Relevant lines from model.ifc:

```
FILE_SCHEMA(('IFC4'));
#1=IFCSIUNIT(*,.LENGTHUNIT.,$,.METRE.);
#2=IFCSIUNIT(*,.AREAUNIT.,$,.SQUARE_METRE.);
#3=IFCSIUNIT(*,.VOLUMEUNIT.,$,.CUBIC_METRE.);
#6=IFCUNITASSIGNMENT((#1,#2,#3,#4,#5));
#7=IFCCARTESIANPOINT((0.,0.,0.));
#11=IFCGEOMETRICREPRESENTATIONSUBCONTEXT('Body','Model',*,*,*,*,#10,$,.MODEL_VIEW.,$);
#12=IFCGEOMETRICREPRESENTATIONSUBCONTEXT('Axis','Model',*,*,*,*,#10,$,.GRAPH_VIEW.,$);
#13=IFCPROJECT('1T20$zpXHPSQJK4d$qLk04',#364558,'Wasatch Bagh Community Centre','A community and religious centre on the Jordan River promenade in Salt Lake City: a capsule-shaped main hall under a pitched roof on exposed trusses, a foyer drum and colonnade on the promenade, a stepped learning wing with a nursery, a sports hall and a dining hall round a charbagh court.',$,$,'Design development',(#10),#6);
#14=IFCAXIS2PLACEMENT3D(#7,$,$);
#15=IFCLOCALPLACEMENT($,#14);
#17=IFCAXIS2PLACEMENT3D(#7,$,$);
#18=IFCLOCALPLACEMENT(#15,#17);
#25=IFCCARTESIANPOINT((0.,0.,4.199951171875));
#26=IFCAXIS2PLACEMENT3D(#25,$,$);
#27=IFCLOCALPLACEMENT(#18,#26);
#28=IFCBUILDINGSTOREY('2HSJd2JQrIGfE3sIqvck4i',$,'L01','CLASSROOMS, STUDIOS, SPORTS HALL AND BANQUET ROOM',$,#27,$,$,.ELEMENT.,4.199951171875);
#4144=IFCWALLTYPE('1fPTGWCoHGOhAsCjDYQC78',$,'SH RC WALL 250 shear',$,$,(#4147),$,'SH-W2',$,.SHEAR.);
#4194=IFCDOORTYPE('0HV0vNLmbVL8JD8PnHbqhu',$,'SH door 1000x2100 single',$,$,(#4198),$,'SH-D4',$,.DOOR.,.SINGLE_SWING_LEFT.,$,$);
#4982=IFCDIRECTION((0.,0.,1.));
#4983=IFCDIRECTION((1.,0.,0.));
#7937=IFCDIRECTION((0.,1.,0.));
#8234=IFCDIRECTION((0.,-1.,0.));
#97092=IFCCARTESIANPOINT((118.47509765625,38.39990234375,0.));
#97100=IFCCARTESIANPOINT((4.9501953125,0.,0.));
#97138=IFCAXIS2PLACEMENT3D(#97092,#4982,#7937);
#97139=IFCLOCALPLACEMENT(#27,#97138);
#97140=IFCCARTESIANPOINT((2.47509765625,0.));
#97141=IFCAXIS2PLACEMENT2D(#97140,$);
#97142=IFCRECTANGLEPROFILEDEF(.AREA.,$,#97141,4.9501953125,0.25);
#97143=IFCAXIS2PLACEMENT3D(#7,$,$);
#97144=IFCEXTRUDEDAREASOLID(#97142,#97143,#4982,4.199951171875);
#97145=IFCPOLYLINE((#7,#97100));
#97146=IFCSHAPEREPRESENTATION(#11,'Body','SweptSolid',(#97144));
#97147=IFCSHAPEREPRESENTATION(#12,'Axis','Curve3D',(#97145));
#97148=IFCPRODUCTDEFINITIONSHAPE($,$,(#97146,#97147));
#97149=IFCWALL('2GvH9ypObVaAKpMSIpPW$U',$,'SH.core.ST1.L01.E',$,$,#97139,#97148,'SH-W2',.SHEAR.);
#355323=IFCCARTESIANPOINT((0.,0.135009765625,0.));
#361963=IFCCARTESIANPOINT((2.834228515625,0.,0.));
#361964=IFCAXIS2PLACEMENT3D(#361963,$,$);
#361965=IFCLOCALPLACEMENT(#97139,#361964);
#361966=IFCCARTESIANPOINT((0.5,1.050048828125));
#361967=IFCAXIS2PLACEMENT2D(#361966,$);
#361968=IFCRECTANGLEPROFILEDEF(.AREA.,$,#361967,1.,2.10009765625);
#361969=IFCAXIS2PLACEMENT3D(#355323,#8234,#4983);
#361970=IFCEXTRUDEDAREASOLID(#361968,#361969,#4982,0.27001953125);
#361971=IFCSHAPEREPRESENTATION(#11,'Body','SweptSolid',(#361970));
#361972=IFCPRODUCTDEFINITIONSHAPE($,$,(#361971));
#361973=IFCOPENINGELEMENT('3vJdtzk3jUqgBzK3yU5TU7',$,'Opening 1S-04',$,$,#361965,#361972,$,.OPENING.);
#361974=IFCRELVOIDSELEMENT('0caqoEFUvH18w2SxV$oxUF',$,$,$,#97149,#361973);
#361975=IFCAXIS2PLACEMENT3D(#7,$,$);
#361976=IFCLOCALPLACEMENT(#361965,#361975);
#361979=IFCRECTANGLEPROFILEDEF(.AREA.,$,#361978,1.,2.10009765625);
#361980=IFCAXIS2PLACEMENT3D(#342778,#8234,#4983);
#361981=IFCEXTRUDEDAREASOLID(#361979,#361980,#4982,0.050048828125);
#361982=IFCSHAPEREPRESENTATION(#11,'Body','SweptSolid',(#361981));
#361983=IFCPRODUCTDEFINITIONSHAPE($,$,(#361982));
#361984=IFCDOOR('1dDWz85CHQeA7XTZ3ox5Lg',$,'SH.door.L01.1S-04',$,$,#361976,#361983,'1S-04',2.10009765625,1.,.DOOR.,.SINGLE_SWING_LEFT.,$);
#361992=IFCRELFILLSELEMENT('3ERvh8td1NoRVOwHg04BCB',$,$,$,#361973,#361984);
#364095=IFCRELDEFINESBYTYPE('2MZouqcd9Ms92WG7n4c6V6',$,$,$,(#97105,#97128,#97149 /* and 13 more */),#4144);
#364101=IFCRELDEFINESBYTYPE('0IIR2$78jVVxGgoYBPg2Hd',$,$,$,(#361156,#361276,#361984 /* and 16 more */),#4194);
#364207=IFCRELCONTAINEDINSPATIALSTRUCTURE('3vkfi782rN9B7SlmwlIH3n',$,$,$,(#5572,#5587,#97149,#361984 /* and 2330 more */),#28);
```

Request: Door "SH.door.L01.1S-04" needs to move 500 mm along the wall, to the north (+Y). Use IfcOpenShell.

```python
import ifcopenshell
import ifcopenshell.api.geometry
import ifcopenshell.util.placement
import ifcopenshell.util.unit

model = ifcopenshell.open("model.ifc")
unit_scale = ifcopenshell.util.unit.calculate_unit_scale(model)

door = model.by_id(361984)
opening = door.FillsVoids[0].RelatingOpeningElement
wall = opening.VoidsElements[0].RelatingBuildingElement

wall_matrix = ifcopenshell.util.placement.get_local_placement(wall.ObjectPlacement)
shift = wall_matrix[:3, 0] * 0.5 / unit_scale
before = ifcopenshell.util.placement.get_local_placement(door.ObjectPlacement)[:3, 3].copy()

# The door is placed relative to its opening, so it follows when the opening moves.
matrix = ifcopenshell.util.placement.get_local_placement(opening.ObjectPlacement)
matrix[:3, 3] += shift
ifcopenshell.api.geometry.edit_object_placement(
    model, product=opening, matrix=matrix, is_si=False, should_transform_children=True
)

after = ifcopenshell.util.placement.get_local_placement(door.ObjectPlacement)[:3, 3]
print("door moved by", (after - before).round(3) + 0.0)

model.write("model_rev.ifc")
```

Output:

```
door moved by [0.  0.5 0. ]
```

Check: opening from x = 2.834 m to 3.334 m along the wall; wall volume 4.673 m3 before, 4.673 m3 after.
